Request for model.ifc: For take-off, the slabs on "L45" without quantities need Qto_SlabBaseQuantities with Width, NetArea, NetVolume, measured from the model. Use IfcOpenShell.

First a look at what the model holds.

```python
import ifcopenshell
import ifcopenshell.util.element
import ifcopenshell.util.unit

model = ifcopenshell.open("model.ifc")
print(model.schema)
for unit_type in ("LENGTHUNIT", "AREAUNIT", "VOLUMEUNIT"):
    print(unit_type, ifcopenshell.util.unit.calculate_unit_scale(model, unit_type))
storey = next(s for s in model.by_type("IfcBuildingStorey") if s.Name == "L45")
slabs = [e for e in ifcopenshell.util.element.get_decomposition(storey) if e.is_a("IfcSlab")]
for e in sorted(slabs, key=lambda e: e.id()):
    print(e.id(), e.is_a(), e.Name, list(ifcopenshell.util.element.get_psets(e, qtos_only=True)), sep=" | ")
```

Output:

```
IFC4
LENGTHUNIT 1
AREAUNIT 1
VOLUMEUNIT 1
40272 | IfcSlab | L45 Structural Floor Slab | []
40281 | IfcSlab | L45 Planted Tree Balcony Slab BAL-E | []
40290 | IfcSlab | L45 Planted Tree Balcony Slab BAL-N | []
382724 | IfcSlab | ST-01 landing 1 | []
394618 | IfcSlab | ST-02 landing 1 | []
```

```python
import ifcopenshell
import ifcopenshell.api.pset
import ifcopenshell.geom
import ifcopenshell.util.element
import ifcopenshell.util.shape
import ifcopenshell.util.unit

model = ifcopenshell.open("model.ifc")
unit_scale = ifcopenshell.util.unit.calculate_unit_scale(model)
area_scale = ifcopenshell.util.unit.calculate_unit_scale(model, "AREAUNIT")
volume_scale = ifcopenshell.util.unit.calculate_unit_scale(model, "VOLUMEUNIT")
settings = ifcopenshell.geom.settings()

storey = next(s for s in model.by_type("IfcBuildingStorey") if s.Name == "L45")
slabs = [e for e in ifcopenshell.util.element.get_decomposition(storey) if e.is_a("IfcSlab")]

for e in sorted(slabs, key=lambda e: e.id()):
    if ifcopenshell.util.element.get_psets(e, qtos_only=True, should_inherit=False):
        continue
    # Geometry comes back in metres, in the element's own axes.
    shape = ifcopenshell.geom.create_shape(settings, e)
    values = {
        "Width": ifcopenshell.util.shape.get_z(shape.geometry) / unit_scale,
        "NetArea": ifcopenshell.util.shape.get_footprint_area(shape.geometry) / area_scale,
        "NetVolume": ifcopenshell.util.shape.get_volume(shape.geometry) / volume_scale,
    }
    qto = ifcopenshell.api.pset.add_qto(model, product=e, name="Qto_SlabBaseQuantities")
    ifcopenshell.api.pset.edit_qto(model, qto=qto, properties=values)
    print(e.id(), {k: round(v, 3) for k, v in values.items()})

model.write("model_updated.ifc")
```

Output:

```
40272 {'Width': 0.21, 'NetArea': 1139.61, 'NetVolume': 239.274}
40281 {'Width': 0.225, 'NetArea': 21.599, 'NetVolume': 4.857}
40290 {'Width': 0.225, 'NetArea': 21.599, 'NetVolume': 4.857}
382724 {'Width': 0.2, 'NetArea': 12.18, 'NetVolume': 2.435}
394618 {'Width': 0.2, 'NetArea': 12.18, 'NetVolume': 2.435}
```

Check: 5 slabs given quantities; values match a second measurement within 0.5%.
